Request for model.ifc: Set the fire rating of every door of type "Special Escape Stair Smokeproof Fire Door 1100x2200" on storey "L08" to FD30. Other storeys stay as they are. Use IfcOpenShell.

First a look at what the model holds.

```python
import ifcopenshell
import ifcopenshell.util.element

model = ifcopenshell.open("model.ifc")
print(model.schema)
storey = next(s for s in model.by_type("IfcBuildingStorey") if s.Name == "L08")
doors = [e for e in ifcopenshell.util.element.get_decomposition(storey) if e.is_a("IfcDoor")]
seen = {}
for e in doors:
    element_type = ifcopenshell.util.element.get_type(e)
    key = (element_type.Name if element_type != e and element_type else None, ifcopenshell.util.element.get_pset(e, "Pset_DoorCommon", "FireRating"))
    seen[key] = seen.get(key, 0) + 1
for (name, value), count in sorted(seen.items(), key=str):
    print(count, "x", name, "|", value)
```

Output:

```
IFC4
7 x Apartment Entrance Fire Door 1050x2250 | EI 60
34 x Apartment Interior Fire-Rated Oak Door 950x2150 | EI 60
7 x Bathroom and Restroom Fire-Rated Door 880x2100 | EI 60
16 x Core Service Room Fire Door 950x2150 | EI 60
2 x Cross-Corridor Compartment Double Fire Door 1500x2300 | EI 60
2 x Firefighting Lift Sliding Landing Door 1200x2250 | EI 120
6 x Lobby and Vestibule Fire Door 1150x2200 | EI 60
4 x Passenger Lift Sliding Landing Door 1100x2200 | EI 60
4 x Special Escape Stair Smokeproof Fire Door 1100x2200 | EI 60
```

```python
import ifcopenshell
import ifcopenshell.api.pset
import ifcopenshell.util.element

model = ifcopenshell.open("model.ifc")

storey = next(s for s in model.by_type("IfcBuildingStorey") if s.Name == "L08")
doors = [e for e in ifcopenshell.util.element.get_decomposition(storey) if e.is_a("IfcDoor")]

count = 0
for e in doors:
    element_type = ifcopenshell.util.element.get_type(e)
    if element_type in (None, e) or element_type.Name != "Special Escape Stair Smokeproof Fire Door 1100x2200":
        continue
    found = ifcopenshell.util.element.get_pset(e, "Pset_DoorCommon", should_inherit=False)
    if found:
        pset = model.by_id(found["id"])
        if len(ifcopenshell.util.element.get_elements_by_pset(pset)) > 1:
            pset = ifcopenshell.api.pset.unshare_pset(model, products=[e], pset=pset)[0]
    else:
        pset = ifcopenshell.api.pset.add_pset(model, product=e, name="Pset_DoorCommon")
    ifcopenshell.api.pset.edit_pset(model, pset=pset, properties={"FireRating": "FD30"})
    count += 1

print(count, "doors updated")

model.write("model_edited.ifc")
```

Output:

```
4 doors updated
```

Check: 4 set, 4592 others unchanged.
